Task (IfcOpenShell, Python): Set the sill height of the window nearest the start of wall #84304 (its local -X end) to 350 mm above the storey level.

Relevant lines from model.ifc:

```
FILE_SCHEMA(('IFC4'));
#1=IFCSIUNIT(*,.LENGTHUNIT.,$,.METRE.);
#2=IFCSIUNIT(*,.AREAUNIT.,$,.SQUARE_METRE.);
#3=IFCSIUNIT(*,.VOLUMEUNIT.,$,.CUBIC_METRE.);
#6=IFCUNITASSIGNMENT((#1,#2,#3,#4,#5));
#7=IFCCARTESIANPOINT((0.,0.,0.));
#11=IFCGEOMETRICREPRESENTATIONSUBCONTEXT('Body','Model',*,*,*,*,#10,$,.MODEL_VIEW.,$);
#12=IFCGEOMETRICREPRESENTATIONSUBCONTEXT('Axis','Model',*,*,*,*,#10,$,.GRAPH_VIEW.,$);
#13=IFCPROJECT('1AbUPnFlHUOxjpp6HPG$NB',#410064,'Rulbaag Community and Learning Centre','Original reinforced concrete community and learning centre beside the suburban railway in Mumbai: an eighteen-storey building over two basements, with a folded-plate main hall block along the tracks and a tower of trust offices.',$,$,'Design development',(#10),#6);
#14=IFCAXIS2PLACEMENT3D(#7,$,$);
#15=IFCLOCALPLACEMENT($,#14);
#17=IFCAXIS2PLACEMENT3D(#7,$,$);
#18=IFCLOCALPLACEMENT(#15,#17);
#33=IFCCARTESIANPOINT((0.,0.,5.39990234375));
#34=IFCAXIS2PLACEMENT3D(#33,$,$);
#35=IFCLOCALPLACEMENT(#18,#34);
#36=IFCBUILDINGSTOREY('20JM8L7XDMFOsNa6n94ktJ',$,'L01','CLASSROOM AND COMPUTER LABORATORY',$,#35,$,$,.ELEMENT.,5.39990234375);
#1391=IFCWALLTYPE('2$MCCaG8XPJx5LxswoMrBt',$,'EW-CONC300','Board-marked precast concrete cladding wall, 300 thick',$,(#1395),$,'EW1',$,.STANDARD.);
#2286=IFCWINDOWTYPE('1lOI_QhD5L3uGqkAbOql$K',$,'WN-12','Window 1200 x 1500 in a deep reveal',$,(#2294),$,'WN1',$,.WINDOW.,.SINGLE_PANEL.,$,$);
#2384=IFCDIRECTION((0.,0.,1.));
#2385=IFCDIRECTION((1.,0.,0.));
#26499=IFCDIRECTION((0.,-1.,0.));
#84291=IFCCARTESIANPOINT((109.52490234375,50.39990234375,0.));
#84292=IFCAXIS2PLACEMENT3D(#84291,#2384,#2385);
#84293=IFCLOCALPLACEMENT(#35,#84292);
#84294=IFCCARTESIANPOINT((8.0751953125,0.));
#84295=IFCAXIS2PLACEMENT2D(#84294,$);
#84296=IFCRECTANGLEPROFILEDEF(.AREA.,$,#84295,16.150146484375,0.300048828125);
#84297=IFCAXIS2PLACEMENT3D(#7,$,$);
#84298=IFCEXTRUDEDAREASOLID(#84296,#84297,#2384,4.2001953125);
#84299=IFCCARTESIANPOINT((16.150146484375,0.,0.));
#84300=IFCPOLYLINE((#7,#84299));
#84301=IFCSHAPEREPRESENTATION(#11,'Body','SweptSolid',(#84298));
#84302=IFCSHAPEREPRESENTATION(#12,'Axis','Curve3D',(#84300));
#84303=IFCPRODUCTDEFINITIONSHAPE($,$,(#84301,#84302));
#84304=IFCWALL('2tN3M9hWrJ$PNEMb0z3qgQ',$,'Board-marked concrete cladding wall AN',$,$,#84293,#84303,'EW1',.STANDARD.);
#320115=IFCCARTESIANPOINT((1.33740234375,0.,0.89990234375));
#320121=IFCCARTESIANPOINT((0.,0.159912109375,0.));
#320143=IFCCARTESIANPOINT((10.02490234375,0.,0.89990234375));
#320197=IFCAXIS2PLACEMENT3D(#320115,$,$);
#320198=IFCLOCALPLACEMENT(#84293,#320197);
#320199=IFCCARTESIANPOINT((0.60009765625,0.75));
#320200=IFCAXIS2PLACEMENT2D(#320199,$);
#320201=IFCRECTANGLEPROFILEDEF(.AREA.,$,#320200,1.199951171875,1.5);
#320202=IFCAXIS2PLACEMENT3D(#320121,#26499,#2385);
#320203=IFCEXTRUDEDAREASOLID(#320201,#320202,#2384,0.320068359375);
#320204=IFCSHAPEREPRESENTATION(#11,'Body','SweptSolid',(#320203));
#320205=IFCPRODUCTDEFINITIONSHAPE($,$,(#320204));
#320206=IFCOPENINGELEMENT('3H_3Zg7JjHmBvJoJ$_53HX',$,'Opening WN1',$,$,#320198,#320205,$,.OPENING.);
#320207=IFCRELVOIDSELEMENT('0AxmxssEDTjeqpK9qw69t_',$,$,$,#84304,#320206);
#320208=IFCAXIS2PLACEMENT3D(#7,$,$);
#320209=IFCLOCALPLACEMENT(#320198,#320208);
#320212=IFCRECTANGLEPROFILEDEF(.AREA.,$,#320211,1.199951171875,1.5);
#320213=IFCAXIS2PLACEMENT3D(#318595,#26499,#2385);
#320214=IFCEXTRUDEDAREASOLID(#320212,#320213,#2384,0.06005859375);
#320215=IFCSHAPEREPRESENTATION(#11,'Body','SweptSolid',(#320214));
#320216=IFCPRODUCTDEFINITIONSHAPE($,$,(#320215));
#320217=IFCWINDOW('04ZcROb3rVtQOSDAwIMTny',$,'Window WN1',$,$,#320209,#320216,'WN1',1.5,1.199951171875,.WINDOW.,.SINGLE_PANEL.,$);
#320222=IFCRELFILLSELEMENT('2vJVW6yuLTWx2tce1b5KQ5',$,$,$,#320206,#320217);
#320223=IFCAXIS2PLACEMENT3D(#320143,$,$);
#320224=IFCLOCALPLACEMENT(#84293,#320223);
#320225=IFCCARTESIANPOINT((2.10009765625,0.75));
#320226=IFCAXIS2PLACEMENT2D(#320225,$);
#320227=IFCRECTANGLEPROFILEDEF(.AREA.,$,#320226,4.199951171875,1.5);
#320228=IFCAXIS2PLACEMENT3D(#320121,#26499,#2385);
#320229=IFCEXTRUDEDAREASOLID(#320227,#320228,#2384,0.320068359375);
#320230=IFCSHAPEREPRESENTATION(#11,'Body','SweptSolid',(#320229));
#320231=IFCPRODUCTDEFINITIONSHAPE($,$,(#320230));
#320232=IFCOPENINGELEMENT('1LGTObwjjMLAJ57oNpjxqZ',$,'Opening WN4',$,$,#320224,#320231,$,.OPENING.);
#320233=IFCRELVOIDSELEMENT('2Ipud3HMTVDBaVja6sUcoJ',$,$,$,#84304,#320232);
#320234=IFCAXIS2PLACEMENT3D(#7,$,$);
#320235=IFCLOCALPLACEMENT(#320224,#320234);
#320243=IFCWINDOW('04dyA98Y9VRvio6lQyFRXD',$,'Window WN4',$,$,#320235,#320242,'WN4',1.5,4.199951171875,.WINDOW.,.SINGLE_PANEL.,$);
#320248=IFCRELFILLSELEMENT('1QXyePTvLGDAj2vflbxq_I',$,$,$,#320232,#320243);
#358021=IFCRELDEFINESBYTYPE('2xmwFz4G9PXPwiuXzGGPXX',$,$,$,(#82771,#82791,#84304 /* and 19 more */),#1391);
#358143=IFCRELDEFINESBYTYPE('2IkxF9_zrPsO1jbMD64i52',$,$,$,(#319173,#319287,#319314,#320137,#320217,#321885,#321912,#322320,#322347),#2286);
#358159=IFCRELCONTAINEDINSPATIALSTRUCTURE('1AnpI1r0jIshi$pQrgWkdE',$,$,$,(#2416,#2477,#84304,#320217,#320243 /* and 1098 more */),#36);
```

```python
import numpy as np
import ifcopenshell
import ifcopenshell.api.geometry
import ifcopenshell.geom
import ifcopenshell.util.element
import ifcopenshell.util.placement
import ifcopenshell.util.shape
import ifcopenshell.util.unit

model = ifcopenshell.open("model.ifc")
unit_scale = ifcopenshell.util.unit.calculate_unit_scale(model)

window = model.by_guid("04ZcROb3rVtQOSDAwIMTny")
opening = window.FillsVoids[0].RelatingOpeningElement
storey = ifcopenshell.util.element.get_container(window, ifc_class="IfcBuildingStorey")
level = ifcopenshell.util.placement.get_local_placement(storey.ObjectPlacement)[2, 3]

# The opening's origin need not be at the sill, so measure its lowest point.
shape = ifcopenshell.geom.create_shape(ifcopenshell.geom.settings(), opening)
bottom = ifcopenshell.util.shape.get_shape_bottom_elevation(shape, shape.geometry) / unit_scale
dz = level + 0.35 / unit_scale - bottom

shift = np.array([0.0, 0.0, dz])
# The window is placed relative to its opening, so it follows when the opening moves.
matrix = ifcopenshell.util.placement.get_local_placement(opening.ObjectPlacement)
matrix[:3, 3] += shift
ifcopenshell.api.geometry.edit_object_placement(
    model, product=opening, matrix=matrix, is_si=False, should_transform_children=True
)

print(f"moved by {dz * unit_scale:+.3f} m")

model.write("model_updated.ifc")
```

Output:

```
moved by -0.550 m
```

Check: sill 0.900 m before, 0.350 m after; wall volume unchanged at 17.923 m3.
